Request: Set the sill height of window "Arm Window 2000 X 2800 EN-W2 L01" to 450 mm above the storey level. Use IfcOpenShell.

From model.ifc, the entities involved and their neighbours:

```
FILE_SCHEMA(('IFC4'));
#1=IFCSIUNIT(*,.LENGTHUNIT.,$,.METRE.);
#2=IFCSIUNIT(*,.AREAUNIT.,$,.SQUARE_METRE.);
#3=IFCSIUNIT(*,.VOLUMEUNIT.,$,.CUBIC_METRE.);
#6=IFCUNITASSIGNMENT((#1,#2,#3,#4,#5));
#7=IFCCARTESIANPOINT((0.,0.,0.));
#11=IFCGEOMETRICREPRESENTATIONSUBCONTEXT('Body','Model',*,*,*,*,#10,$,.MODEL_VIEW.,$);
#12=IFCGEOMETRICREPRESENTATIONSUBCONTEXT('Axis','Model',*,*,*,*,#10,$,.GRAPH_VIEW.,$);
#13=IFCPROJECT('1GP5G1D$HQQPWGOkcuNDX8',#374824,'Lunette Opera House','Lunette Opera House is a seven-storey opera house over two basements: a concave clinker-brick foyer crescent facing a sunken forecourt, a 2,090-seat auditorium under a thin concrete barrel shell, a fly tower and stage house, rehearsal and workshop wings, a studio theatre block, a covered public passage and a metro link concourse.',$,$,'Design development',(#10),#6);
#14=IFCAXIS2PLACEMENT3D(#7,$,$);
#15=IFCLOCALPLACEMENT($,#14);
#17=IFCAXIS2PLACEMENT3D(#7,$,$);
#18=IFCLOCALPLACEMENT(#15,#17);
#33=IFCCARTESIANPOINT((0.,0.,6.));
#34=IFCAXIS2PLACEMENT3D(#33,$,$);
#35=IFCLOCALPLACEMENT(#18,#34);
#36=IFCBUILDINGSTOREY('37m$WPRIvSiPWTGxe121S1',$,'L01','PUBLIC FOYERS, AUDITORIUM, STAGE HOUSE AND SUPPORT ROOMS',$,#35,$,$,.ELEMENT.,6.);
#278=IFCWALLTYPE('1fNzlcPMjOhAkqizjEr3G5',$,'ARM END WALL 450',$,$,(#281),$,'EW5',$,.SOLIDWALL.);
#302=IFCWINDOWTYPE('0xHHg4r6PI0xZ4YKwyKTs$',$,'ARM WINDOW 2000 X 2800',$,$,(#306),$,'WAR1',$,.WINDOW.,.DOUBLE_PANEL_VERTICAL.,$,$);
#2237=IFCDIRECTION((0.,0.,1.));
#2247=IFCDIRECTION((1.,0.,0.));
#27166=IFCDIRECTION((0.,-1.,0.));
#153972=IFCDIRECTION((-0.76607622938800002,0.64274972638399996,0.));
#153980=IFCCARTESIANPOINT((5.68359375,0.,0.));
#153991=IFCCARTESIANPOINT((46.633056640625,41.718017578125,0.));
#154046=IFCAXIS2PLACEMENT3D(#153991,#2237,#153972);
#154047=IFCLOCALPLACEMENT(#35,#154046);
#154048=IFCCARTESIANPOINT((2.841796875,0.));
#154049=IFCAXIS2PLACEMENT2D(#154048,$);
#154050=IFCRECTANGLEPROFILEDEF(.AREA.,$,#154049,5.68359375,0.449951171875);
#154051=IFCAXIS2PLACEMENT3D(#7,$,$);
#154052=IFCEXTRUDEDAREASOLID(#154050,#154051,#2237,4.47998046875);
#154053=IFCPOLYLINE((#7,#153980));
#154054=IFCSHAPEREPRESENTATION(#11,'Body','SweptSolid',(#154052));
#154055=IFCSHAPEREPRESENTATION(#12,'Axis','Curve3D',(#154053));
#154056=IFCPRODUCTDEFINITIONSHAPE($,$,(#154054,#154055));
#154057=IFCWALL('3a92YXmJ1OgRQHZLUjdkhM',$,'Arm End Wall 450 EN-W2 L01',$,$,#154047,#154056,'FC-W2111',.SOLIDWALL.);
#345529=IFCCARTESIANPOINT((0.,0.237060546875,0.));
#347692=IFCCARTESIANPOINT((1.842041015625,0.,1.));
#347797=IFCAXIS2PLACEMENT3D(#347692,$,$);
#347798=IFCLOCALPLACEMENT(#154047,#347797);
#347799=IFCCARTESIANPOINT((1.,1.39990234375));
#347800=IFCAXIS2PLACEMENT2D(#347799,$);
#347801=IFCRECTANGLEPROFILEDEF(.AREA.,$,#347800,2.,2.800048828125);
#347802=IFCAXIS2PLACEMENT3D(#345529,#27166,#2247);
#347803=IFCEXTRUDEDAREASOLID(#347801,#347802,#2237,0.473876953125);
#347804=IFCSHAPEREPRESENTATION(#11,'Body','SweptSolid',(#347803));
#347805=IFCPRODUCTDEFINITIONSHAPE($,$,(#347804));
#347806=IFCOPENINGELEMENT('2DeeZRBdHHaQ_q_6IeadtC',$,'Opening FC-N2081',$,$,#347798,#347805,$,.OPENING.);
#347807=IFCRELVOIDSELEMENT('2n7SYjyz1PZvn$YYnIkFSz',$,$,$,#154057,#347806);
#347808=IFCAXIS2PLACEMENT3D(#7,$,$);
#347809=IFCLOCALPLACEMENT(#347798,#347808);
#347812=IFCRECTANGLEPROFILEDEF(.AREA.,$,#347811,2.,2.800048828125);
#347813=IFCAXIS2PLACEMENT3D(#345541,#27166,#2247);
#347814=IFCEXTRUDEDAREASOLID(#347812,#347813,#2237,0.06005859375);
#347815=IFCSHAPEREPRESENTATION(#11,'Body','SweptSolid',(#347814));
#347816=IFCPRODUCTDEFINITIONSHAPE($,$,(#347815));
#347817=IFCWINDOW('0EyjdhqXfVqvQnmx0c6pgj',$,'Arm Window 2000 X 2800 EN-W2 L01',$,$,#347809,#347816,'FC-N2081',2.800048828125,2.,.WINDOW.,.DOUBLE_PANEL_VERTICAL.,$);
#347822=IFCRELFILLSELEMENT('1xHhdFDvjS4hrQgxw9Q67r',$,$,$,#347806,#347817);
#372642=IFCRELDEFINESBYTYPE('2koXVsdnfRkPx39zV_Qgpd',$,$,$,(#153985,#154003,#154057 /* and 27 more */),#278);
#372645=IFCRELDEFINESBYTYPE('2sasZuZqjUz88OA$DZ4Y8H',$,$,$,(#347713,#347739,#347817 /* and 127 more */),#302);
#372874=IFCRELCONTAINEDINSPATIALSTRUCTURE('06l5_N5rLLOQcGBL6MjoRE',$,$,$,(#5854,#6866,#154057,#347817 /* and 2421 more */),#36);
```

```python
import numpy as np
import ifcopenshell
import ifcopenshell.api.geometry
import ifcopenshell.geom
import ifcopenshell.util.element
import ifcopenshell.util.placement
import ifcopenshell.util.shape
import ifcopenshell.util.unit

model = ifcopenshell.open("model.ifc")
unit_scale = ifcopenshell.util.unit.calculate_unit_scale(model)

window = model.by_id(347817)
opening = window.FillsVoids[0].RelatingOpeningElement
storey = ifcopenshell.util.element.get_container(window, ifc_class="IfcBuildingStorey")
level = ifcopenshell.util.placement.get_local_placement(storey.ObjectPlacement)[2, 3]

# The opening's origin need not be at the sill, so measure its lowest point.
shape = ifcopenshell.geom.create_shape(ifcopenshell.geom.settings(), opening)
bottom = ifcopenshell.util.shape.get_shape_bottom_elevation(shape, shape.geometry) / unit_scale
dz = level + 0.45 / unit_scale - bottom

shift = np.array([0.0, 0.0, dz])
# The window is placed relative to its opening, so it follows when the opening moves.
matrix = ifcopenshell.util.placement.get_local_placement(opening.ObjectPlacement)
matrix[:3, 3] += shift
ifcopenshell.api.geometry.edit_object_placement(
    model, product=opening, matrix=matrix, is_si=False, should_transform_children=True
)

print(f"moved by {dz * unit_scale:+.3f} m")

model.write("model_v2.ifc")
```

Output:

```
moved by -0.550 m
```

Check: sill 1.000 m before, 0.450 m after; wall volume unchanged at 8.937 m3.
